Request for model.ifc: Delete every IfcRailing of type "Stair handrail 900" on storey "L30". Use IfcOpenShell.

First a look at what the model holds.

```python
import ifcopenshell
import ifcopenshell.util.element

model = ifcopenshell.open("model.ifc")
print(model.schema)
storey = next(s for s in model.by_type("IfcBuildingStorey") if s.Name == "L30")
railings = [e for e in ifcopenshell.util.element.get_decomposition(storey) if e.is_a("IfcRailing")]
seen = {}
for e in railings:
    element_type = ifcopenshell.util.element.get_type(e)
    name = element_type.Name if element_type not in (None, e) else None
    seen[name] = seen.get(name, 0) + 1
for name, count in sorted(seen.items(), key=str):
    print(count, "x", name)
```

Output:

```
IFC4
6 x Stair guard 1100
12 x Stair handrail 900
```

```python
import ifcopenshell
import ifcopenshell.api.root
import ifcopenshell.util.element

model = ifcopenshell.open("model.ifc")

storey = next(s for s in model.by_type("IfcBuildingStorey") if s.Name == "L30")
railings = [e for e in ifcopenshell.util.element.get_decomposition(storey) if e.is_a("IfcRailing")]
targets = [e for e in railings if (t := ifcopenshell.util.element.get_type(e)) not in (None, e) and t.Name == "Stair handrail 900"]

for e in targets:
    ifcopenshell.api.root.remove_product(model, product=e)
print(len(targets), "removed")

model.write("model_edited.ifc")
```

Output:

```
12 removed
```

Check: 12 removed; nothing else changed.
